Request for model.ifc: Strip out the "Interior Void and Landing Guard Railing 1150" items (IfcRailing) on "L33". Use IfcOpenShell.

First a look at what the model holds.

```python
import ifcopenshell
import ifcopenshell.util.element

model = ifcopenshell.open("model.ifc")
print(model.schema)
storey = next(s for s in model.by_type("IfcBuildingStorey") if s.Name == "L33")
railings = [e for e in ifcopenshell.util.element.get_decomposition(storey) if e.is_a("IfcRailing")]
seen = {}
for e in railings:
    element_type = ifcopenshell.util.element.get_type(e)
    name = element_type.Name if element_type not in (None, e) else None
    seen[name] = seen.get(name, 0) + 1
for name, count in sorted(seen.items(), key=str):
    print(count, "x", name)
```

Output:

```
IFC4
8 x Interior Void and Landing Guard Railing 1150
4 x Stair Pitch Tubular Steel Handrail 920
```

```python
import ifcopenshell
import ifcopenshell.api.root
import ifcopenshell.util.element

model = ifcopenshell.open("model.ifc")

storey = next(s for s in model.by_type("IfcBuildingStorey") if s.Name == "L33")
railings = [e for e in ifcopenshell.util.element.get_decomposition(storey) if e.is_a("IfcRailing")]
targets = [e for e in railings if (t := ifcopenshell.util.element.get_type(e)) not in (None, e) and t.Name == "Interior Void and Landing Guard Railing 1150"]

for e in targets:
    ifcopenshell.api.root.remove_product(model, product=e)
print(len(targets), "removed")

model.write("model_v2.ifc")
```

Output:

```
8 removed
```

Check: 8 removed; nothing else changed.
